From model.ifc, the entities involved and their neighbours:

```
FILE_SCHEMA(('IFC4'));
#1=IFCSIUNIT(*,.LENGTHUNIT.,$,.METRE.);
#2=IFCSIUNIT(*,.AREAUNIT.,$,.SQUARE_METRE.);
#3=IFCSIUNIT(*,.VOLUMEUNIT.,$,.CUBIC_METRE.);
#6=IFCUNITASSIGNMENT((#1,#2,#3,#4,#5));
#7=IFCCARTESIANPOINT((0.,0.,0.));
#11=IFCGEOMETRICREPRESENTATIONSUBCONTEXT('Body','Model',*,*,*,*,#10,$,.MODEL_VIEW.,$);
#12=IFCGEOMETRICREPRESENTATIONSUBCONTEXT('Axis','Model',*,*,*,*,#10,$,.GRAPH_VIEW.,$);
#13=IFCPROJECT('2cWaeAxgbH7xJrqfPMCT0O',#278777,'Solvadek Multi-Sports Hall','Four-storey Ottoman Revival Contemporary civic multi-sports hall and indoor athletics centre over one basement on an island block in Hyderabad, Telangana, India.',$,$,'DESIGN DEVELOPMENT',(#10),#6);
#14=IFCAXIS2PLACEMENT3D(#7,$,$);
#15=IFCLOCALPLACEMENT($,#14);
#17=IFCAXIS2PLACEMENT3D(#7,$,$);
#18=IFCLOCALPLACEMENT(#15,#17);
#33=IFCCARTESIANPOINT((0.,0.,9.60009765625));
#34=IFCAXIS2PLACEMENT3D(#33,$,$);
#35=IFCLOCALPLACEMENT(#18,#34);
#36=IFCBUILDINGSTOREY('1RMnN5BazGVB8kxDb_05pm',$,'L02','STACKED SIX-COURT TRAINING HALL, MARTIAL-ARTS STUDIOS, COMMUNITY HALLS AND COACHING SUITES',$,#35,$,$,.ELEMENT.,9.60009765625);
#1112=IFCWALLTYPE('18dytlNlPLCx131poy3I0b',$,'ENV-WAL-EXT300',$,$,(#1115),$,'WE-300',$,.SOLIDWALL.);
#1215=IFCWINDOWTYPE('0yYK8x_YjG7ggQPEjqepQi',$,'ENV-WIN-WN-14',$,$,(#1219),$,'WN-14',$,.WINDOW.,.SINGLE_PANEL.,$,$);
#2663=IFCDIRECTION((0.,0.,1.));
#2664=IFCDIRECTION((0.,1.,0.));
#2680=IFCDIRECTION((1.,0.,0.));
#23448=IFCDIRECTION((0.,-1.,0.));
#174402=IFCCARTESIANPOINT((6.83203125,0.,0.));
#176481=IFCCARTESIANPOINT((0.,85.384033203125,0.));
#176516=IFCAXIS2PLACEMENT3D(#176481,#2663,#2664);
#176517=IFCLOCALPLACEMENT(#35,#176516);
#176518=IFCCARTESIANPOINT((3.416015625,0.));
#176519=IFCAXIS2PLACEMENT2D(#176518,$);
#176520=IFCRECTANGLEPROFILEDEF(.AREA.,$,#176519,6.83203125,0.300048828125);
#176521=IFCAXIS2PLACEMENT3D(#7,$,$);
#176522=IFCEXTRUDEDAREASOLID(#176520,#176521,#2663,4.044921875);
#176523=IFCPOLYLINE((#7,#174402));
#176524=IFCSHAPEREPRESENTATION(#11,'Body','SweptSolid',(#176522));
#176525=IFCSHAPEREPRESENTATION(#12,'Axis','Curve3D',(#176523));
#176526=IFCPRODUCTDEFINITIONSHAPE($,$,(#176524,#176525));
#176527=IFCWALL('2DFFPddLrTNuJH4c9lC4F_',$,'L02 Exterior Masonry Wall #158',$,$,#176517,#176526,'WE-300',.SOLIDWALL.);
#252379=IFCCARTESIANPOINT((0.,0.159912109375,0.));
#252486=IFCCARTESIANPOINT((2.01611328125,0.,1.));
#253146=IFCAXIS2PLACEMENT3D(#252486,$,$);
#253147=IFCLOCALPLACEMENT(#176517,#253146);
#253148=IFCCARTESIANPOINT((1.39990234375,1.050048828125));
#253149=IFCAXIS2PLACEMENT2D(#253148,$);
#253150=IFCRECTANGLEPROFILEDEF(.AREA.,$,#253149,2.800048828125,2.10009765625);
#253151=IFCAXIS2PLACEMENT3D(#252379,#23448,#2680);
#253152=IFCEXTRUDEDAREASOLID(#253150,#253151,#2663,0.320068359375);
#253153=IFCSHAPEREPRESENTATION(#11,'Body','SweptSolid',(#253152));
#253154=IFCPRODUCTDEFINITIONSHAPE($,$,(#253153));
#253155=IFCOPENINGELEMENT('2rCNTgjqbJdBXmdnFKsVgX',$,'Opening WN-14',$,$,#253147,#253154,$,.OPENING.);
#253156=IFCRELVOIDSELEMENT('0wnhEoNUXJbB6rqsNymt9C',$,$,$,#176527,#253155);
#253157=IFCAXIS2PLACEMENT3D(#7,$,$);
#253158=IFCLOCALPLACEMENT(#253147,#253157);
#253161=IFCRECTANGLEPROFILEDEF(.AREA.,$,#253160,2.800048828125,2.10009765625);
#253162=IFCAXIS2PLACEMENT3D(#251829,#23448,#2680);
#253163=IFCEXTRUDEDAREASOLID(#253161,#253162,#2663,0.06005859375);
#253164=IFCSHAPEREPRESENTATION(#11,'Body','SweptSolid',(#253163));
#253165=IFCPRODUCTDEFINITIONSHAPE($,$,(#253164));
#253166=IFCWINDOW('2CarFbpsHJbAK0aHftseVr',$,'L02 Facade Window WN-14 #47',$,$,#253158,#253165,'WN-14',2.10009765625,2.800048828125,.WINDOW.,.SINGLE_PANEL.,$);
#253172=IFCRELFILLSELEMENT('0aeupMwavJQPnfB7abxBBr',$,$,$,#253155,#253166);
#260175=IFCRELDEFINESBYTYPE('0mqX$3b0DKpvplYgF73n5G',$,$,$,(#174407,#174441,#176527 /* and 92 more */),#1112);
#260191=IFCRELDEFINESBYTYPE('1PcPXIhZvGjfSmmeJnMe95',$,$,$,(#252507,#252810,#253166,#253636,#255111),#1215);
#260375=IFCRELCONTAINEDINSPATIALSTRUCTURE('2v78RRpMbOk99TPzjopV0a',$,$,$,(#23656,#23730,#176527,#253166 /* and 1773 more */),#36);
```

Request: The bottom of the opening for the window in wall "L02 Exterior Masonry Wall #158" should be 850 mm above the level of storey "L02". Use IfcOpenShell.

```python
import numpy as np
import ifcopenshell
import ifcopenshell.api.geometry
import ifcopenshell.geom
import ifcopenshell.util.element
import ifcopenshell.util.placement
import ifcopenshell.util.shape
import ifcopenshell.util.unit

model = ifcopenshell.open("model.ifc")
unit_scale = ifcopenshell.util.unit.calculate_unit_scale(model)

window = model.by_guid("2CarFbpsHJbAK0aHftseVr")
opening = window.FillsVoids[0].RelatingOpeningElement
storey = ifcopenshell.util.element.get_container(window, ifc_class="IfcBuildingStorey")
level = ifcopenshell.util.placement.get_local_placement(storey.ObjectPlacement)[2, 3]

# The opening's origin need not be at the sill, so measure its lowest point.
shape = ifcopenshell.geom.create_shape(ifcopenshell.geom.settings(), opening)
bottom = ifcopenshell.util.shape.get_shape_bottom_elevation(shape, shape.geometry) / unit_scale
dz = level + 0.85 - bottom

shift = np.array([0.0, 0.0, dz])
# The window is placed relative to its opening, so it follows when the opening moves.
matrix = ifcopenshell.util.placement.get_local_placement(opening.ObjectPlacement)
matrix[:3, 3] += shift
ifcopenshell.api.geometry.edit_object_placement(
    model, product=opening, matrix=matrix, is_si=False, should_transform_children=True
)

print(f"moved by {dz * unit_scale:+.3f} m")

model.write("model_v2.ifc")
```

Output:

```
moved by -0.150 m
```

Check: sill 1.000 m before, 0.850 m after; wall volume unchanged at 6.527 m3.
